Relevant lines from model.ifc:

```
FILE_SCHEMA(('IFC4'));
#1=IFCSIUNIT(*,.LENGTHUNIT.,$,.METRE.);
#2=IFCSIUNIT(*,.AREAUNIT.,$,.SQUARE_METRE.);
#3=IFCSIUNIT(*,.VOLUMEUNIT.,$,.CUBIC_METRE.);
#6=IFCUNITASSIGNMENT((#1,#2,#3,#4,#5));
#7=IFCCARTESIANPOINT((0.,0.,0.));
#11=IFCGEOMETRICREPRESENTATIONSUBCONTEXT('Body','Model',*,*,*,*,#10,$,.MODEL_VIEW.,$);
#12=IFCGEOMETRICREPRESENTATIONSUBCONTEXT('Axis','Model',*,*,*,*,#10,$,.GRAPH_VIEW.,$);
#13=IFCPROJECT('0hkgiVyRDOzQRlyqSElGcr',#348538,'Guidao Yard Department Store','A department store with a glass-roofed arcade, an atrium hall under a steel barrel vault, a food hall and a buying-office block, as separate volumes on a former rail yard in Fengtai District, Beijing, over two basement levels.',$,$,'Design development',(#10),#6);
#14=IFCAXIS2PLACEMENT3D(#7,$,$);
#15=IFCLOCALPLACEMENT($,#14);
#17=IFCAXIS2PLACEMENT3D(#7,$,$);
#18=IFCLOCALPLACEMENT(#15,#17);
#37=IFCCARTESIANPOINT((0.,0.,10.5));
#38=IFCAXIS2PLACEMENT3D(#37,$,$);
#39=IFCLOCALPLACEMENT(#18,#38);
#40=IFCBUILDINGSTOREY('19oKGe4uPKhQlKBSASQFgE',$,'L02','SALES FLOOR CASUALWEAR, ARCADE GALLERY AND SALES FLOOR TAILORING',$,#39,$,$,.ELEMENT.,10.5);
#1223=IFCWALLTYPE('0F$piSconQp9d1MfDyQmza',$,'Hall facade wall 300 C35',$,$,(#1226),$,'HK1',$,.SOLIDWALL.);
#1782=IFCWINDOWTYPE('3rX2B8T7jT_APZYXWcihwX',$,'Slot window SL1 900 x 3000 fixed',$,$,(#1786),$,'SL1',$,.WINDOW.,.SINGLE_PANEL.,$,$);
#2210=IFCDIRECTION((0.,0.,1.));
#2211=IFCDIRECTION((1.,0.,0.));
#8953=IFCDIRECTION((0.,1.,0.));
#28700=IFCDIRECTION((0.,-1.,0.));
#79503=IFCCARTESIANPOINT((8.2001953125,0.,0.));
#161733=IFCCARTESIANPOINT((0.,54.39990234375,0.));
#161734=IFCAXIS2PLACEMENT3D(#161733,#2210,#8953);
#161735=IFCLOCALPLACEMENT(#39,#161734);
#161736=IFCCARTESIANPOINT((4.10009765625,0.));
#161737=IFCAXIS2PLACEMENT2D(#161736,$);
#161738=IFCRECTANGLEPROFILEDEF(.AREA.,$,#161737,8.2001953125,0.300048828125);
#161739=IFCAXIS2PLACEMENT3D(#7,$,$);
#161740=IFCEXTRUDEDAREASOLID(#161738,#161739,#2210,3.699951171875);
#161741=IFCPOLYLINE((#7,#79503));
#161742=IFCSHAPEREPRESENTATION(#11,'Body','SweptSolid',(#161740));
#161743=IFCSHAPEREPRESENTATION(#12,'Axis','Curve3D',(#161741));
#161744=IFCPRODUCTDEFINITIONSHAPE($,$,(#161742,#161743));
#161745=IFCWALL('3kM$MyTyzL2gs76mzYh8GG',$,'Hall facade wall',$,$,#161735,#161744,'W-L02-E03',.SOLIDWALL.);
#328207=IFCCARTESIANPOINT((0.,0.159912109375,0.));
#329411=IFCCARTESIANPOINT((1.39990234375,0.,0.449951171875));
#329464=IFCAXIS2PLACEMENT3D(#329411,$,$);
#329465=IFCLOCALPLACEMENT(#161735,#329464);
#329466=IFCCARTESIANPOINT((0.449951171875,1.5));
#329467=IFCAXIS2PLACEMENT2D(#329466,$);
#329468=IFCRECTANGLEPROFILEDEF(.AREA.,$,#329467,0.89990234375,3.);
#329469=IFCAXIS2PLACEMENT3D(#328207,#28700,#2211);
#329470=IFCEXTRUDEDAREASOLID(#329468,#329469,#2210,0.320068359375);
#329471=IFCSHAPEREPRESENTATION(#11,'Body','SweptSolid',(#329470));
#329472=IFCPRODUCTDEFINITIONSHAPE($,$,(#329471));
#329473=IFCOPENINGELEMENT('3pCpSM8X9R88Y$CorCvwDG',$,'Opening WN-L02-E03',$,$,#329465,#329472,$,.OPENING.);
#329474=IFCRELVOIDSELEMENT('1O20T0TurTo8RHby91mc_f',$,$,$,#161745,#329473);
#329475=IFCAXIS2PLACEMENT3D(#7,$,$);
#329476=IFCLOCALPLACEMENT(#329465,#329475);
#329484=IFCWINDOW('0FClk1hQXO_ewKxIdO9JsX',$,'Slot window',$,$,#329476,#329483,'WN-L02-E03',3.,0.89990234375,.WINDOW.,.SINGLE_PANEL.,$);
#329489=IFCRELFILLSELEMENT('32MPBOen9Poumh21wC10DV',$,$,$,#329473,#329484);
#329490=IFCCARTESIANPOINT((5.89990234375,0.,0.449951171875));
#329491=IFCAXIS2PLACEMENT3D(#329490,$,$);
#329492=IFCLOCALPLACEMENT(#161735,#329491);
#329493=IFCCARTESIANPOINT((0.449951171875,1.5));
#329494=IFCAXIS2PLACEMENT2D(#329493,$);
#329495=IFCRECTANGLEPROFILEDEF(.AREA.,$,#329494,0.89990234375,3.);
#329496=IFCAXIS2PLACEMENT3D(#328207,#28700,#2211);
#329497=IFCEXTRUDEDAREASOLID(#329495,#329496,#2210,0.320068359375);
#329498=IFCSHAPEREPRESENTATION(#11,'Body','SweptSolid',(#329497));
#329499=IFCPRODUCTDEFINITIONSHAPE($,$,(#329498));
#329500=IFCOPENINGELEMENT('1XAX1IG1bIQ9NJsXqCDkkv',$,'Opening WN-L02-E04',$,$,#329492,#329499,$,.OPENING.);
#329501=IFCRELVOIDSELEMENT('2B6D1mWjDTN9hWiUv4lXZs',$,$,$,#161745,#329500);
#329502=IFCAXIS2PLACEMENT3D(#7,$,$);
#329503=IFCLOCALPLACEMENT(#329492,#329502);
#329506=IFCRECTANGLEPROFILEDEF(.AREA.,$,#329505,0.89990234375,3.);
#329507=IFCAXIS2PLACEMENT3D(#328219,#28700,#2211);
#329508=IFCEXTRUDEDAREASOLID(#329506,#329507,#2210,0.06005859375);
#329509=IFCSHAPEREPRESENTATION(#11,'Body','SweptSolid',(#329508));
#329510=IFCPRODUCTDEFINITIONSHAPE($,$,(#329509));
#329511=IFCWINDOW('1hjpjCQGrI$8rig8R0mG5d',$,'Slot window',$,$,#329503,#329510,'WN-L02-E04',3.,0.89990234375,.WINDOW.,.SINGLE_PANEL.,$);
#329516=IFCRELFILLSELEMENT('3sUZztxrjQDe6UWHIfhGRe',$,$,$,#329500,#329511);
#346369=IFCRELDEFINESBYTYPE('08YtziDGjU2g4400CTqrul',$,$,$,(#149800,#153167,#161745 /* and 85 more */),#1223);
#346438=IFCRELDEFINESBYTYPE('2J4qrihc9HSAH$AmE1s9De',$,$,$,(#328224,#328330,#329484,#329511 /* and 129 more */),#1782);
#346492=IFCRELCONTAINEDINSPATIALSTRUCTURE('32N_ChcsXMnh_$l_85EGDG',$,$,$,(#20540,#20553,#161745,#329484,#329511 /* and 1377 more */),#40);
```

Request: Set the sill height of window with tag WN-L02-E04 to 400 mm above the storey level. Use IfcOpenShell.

```python
import numpy as np
import ifcopenshell
import ifcopenshell.api.geometry
import ifcopenshell.geom
import ifcopenshell.util.element
import ifcopenshell.util.placement
import ifcopenshell.util.shape
import ifcopenshell.util.unit

model = ifcopenshell.open("model.ifc")
unit_scale = ifcopenshell.util.unit.calculate_unit_scale(model)

window = model.by_id(329511)
opening = window.FillsVoids[0].RelatingOpeningElement
storey = ifcopenshell.util.element.get_container(window, ifc_class="IfcBuildingStorey")
level = ifcopenshell.util.placement.get_local_placement(storey.ObjectPlacement)[2, 3]

# The opening's origin need not be at the sill, so measure its lowest point.
shape = ifcopenshell.geom.create_shape(ifcopenshell.geom.settings(), opening)
bottom = ifcopenshell.util.shape.get_shape_bottom_elevation(shape, shape.geometry) / unit_scale
dz = level + 0.4 / unit_scale - bottom

shift = np.array([0.0, 0.0, dz])
# The window is placed relative to its opening, so it follows when the opening moves.
matrix = ifcopenshell.util.placement.get_local_placement(opening.ObjectPlacement)
matrix[:3, 3] += shift
ifcopenshell.api.geometry.edit_object_placement(
    model, product=opening, matrix=matrix, is_si=False, should_transform_children=True
)

print(f"moved by {dz * unit_scale:+.3f} m")

model.write("model_updated.ifc")
```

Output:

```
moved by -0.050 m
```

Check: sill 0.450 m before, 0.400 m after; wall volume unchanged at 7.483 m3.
